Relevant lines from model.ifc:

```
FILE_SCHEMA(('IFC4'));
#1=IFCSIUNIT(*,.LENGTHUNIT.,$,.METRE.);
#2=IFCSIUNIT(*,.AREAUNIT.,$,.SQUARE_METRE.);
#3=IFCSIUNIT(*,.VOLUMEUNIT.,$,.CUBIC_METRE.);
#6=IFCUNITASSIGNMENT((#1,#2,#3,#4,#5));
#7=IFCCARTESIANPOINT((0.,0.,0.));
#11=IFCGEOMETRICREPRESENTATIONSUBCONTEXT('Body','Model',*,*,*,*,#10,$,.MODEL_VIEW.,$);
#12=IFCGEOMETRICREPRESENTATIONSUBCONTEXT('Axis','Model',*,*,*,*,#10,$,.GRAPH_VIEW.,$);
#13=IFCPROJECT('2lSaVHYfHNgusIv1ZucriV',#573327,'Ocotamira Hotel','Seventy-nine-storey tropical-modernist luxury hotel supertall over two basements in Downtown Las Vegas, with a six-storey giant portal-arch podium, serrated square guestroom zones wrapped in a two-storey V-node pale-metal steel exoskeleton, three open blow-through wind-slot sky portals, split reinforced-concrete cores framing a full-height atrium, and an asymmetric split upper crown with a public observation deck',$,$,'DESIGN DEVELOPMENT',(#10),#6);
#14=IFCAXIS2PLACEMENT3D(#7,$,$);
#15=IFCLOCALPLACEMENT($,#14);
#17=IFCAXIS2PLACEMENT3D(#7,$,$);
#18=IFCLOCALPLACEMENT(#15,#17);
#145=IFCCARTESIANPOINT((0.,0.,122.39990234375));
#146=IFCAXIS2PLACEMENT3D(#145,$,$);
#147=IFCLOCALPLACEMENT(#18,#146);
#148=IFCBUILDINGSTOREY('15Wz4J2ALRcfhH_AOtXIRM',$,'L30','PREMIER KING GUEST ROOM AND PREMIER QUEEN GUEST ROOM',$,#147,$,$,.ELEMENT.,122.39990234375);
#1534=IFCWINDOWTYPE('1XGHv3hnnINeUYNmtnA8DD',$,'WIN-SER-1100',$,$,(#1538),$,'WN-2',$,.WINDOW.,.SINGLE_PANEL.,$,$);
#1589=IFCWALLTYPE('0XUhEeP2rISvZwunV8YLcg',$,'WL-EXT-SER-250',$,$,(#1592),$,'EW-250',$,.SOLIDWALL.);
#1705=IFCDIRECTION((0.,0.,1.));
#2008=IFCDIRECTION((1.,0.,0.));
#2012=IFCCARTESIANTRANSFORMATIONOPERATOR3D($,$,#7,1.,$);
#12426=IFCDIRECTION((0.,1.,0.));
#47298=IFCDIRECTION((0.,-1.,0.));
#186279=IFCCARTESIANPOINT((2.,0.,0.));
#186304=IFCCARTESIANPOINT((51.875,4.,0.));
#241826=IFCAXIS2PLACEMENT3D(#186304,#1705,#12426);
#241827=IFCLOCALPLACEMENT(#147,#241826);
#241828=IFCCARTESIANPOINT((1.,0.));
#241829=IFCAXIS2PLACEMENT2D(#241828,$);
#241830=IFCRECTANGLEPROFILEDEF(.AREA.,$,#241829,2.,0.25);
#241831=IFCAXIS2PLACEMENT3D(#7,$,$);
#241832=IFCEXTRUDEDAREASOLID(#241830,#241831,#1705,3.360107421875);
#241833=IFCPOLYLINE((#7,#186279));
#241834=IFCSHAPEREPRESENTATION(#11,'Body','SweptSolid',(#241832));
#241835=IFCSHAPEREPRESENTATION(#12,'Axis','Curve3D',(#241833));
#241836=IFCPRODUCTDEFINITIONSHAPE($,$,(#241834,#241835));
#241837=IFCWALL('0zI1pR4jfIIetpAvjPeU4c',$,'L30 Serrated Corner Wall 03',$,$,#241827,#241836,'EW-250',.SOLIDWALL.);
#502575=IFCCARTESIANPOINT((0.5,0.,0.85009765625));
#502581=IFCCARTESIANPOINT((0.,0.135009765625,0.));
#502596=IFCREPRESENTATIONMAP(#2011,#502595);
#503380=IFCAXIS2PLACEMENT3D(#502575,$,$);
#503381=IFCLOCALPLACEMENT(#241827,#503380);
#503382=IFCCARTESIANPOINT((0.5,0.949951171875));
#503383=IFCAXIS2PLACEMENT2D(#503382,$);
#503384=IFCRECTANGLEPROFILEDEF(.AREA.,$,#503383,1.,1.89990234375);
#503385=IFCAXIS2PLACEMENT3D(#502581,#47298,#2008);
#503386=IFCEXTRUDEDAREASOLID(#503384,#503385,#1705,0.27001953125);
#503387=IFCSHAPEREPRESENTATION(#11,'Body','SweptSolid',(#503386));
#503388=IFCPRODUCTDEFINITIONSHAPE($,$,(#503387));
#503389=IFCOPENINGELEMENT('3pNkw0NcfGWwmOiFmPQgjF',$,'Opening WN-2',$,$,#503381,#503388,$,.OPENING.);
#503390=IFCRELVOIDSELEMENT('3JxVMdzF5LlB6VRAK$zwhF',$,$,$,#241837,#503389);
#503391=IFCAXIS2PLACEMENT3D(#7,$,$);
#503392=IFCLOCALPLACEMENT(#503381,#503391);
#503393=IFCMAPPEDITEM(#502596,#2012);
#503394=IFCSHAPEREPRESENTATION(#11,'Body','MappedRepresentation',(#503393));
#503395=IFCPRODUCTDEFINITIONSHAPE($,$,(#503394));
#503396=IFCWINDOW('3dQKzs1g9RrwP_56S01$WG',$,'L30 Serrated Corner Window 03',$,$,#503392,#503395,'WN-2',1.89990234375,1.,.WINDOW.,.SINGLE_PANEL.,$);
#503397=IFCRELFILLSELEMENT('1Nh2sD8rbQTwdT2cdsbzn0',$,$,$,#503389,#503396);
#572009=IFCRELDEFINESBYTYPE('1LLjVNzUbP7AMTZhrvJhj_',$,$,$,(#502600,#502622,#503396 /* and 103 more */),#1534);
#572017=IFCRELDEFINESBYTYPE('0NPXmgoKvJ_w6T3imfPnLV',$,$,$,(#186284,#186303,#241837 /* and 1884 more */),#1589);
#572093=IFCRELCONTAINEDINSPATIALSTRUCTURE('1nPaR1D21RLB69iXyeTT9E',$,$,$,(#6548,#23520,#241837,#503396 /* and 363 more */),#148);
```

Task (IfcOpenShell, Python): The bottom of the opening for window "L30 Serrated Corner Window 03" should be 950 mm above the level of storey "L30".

```python
import numpy as np
import ifcopenshell
import ifcopenshell.api.geometry
import ifcopenshell.geom
import ifcopenshell.util.element
import ifcopenshell.util.placement
import ifcopenshell.util.shape
import ifcopenshell.util.unit

model = ifcopenshell.open("model.ifc")
unit_scale = ifcopenshell.util.unit.calculate_unit_scale(model)

window = model.by_id(503396)
opening = window.FillsVoids[0].RelatingOpeningElement
storey = ifcopenshell.util.element.get_container(window, ifc_class="IfcBuildingStorey")
level = ifcopenshell.util.placement.get_local_placement(storey.ObjectPlacement)[2, 3]

# The opening's origin need not be at the sill, so measure its lowest point.
shape = ifcopenshell.geom.create_shape(ifcopenshell.geom.settings(), opening)
bottom = ifcopenshell.util.shape.get_shape_bottom_elevation(shape, shape.geometry) / unit_scale
dz = level + 0.95 - bottom

shift = np.array([0.0, 0.0, dz])
# The window is placed relative to its opening, so it follows when the opening moves.
matrix = ifcopenshell.util.placement.get_local_placement(opening.ObjectPlacement)
matrix[:3, 3] += shift
ifcopenshell.api.geometry.edit_object_placement(
    model, product=opening, matrix=matrix, is_si=False, should_transform_children=True
)

print(f"moved by {dz * unit_scale:+.3f} m")

model.write("model_edited.ifc")
```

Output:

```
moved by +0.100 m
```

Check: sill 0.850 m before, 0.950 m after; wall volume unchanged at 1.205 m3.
